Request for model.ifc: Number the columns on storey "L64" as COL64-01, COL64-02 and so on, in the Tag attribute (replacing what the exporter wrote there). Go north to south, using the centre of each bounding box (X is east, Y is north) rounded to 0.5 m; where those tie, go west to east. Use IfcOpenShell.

First a look at what the model holds.

```python
import ifcopenshell
import ifcopenshell.util.element
import ifcopenshell.util.placement

model = ifcopenshell.open("model.ifc")
print(model.schema)
storey = next(s for s in model.by_type("IfcBuildingStorey") if s.Name == "L64")
columns = [e for e in ifcopenshell.util.element.get_decomposition(storey) if e.is_a("IfcColumn")]
for e in sorted(columns, key=lambda e: e.id()):
    origin = ifcopenshell.util.placement.get_local_placement(e.ObjectPlacement)[:3, 3]
    print(e.id(), e.Tag, e.Name, origin.round(2) + 0.0, sep=" | ")
```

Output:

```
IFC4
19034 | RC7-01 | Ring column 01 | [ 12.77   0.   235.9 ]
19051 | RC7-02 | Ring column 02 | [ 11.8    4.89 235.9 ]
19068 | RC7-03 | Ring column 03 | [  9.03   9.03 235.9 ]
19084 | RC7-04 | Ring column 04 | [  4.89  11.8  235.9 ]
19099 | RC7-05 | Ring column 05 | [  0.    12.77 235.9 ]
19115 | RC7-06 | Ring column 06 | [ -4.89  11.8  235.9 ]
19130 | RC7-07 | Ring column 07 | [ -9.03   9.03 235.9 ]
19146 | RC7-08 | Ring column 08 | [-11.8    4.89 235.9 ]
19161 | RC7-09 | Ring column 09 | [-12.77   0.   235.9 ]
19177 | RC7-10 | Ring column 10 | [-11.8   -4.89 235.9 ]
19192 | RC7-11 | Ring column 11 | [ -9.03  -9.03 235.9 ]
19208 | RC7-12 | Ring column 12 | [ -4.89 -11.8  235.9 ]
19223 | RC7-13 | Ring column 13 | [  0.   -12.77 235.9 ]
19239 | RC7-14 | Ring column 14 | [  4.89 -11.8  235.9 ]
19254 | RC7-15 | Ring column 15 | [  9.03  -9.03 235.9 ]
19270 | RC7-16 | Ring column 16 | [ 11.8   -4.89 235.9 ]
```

```python
import ifcopenshell
import ifcopenshell.geom
import ifcopenshell.util.element
import ifcopenshell.util.shape

model = ifcopenshell.open("model.ifc")
settings = ifcopenshell.geom.settings()
settings.set("use-world-coords", True)


def centre(element):
    shape = ifcopenshell.geom.create_shape(settings, element)
    return ifcopenshell.util.shape.get_bbox_centroid(shape.geometry)


storey = next(s for s in model.by_type("IfcBuildingStorey") if s.Name == "L64")
columns = [e for e in ifcopenshell.util.element.get_decomposition(storey) if e.is_a("IfcColumn")]

# Insertion points can sit at a corner or the storey origin, so sort by the geometry (in metres).
centres = {e: centre(e) for e in columns}
columns.sort(key=lambda e: (-round(centres[e][1] / 0.5), centres[e][0]))

for i, e in enumerate(columns, start=1):
    number = f"COL64-{i:02d}"
    e.Tag = number
    print(e.id(), number)

model.write("model_v2.ifc")
```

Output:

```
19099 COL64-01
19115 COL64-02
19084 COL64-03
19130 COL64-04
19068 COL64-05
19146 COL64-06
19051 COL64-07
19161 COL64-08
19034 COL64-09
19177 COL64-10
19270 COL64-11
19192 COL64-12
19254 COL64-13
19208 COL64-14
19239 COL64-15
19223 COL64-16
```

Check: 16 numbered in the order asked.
